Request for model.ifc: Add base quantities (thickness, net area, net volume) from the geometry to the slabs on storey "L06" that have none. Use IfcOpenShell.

First a look at what the model holds.

```python
import ifcopenshell
import ifcopenshell.util.element
import ifcopenshell.util.unit

model = ifcopenshell.open("model.ifc")
print(model.schema)
for unit_type in ("LENGTHUNIT", "AREAUNIT", "VOLUMEUNIT"):
    print(unit_type, ifcopenshell.util.unit.calculate_unit_scale(model, unit_type))
storey = next(s for s in model.by_type("IfcBuildingStorey") if s.Name == "L06")
slabs = [e for e in ifcopenshell.util.element.get_decomposition(storey) if e.is_a("IfcSlab")]
for e in sorted(slabs, key=lambda e: e.id()):
    print(e.id(), e.is_a(), e.Name, list(ifcopenshell.util.element.get_psets(e, qtos_only=True)), sep=" | ")
```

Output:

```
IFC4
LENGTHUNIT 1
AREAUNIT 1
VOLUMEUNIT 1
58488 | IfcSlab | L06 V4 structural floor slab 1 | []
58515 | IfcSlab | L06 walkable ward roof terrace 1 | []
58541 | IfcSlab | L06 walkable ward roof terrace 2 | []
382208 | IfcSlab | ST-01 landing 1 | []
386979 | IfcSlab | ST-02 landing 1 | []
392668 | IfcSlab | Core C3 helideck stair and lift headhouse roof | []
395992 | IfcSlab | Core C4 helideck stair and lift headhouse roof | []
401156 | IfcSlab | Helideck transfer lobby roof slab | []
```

```python
import ifcopenshell
import ifcopenshell.api.pset
import ifcopenshell.geom
import ifcopenshell.util.element
import ifcopenshell.util.shape
import ifcopenshell.util.unit

model = ifcopenshell.open("model.ifc")
unit_scale = ifcopenshell.util.unit.calculate_unit_scale(model)
area_scale = ifcopenshell.util.unit.calculate_unit_scale(model, "AREAUNIT")
volume_scale = ifcopenshell.util.unit.calculate_unit_scale(model, "VOLUMEUNIT")
settings = ifcopenshell.geom.settings()

storey = next(s for s in model.by_type("IfcBuildingStorey") if s.Name == "L06")
slabs = [e for e in ifcopenshell.util.element.get_decomposition(storey) if e.is_a("IfcSlab")]

for e in sorted(slabs, key=lambda e: e.id()):
    if ifcopenshell.util.element.get_psets(e, qtos_only=True, should_inherit=False):
        continue
    # Geometry comes back in metres, in the element's own axes.
    shape = ifcopenshell.geom.create_shape(settings, e)
    values = {
        "Width": ifcopenshell.util.shape.get_z(shape.geometry) / unit_scale,
        "NetArea": ifcopenshell.util.shape.get_footprint_area(shape.geometry) / area_scale,
        "NetVolume": ifcopenshell.util.shape.get_volume(shape.geometry) / volume_scale,
    }
    qto = ifcopenshell.api.pset.add_qto(model, product=e, name="Qto_SlabBaseQuantities")
    ifcopenshell.api.pset.edit_qto(model, qto=qto, properties=values)
    print(e.id(), {k: round(v, 3) for k, v in values.items()})

model.write("model_edited.ifc")
```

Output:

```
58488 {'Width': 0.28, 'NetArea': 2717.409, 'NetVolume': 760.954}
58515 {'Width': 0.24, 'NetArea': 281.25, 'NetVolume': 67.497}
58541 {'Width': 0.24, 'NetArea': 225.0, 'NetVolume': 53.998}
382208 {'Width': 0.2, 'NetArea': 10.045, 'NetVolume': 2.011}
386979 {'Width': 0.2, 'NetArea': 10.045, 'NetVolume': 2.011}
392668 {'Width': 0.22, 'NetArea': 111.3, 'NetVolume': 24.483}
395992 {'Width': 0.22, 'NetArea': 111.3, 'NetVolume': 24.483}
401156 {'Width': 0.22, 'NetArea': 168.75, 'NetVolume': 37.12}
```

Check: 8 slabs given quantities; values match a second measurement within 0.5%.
